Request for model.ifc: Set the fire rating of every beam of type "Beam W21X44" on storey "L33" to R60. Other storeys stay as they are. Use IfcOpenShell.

First a look at what the model holds.

```python
import ifcopenshell
import ifcopenshell.util.element

model = ifcopenshell.open("model.ifc")
print(model.schema)
storey = next(s for s in model.by_type("IfcBuildingStorey") if s.Name == "L33")
beams = [e for e in ifcopenshell.util.element.get_decomposition(storey) if e.is_a("IfcBeam")]
seen = {}
for e in beams:
    element_type = ifcopenshell.util.element.get_type(e)
    key = (element_type.Name if element_type != e and element_type else None, ifcopenshell.util.element.get_pset(e, "Pset_BeamCommon", "FireRating"))
    seen[key] = seen.get(key, 0) + 1
for (name, value), count in sorted(seen.items(), key=str):
    print(count, "x", name, "|", value)
```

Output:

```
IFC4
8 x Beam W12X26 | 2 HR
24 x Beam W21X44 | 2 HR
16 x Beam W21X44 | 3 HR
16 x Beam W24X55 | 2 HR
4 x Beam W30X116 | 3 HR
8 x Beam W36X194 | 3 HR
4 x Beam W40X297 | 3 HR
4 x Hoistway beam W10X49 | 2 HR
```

```python
import ifcopenshell
import ifcopenshell.api.pset
import ifcopenshell.util.element

model = ifcopenshell.open("model.ifc")

storey = next(s for s in model.by_type("IfcBuildingStorey") if s.Name == "L33")
beams = [e for e in ifcopenshell.util.element.get_decomposition(storey) if e.is_a("IfcBeam")]

count = 0
for e in beams:
    element_type = ifcopenshell.util.element.get_type(e)
    if element_type in (None, e) or element_type.Name != "Beam W21X44":
        continue
    found = ifcopenshell.util.element.get_pset(e, "Pset_BeamCommon", should_inherit=False)
    if found:
        pset = model.by_id(found["id"])
        if len(ifcopenshell.util.element.get_elements_by_pset(pset)) > 1:
            pset = ifcopenshell.api.pset.unshare_pset(model, products=[e], pset=pset)[0]
    else:
        pset = ifcopenshell.api.pset.add_pset(model, product=e, name="Pset_BeamCommon")
    ifcopenshell.api.pset.edit_pset(model, pset=pset, properties={"FireRating": "R60"})
    count += 1

print(count, "beams updated")

model.write("model_v2.ifc")
```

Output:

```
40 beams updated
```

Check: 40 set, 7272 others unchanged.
